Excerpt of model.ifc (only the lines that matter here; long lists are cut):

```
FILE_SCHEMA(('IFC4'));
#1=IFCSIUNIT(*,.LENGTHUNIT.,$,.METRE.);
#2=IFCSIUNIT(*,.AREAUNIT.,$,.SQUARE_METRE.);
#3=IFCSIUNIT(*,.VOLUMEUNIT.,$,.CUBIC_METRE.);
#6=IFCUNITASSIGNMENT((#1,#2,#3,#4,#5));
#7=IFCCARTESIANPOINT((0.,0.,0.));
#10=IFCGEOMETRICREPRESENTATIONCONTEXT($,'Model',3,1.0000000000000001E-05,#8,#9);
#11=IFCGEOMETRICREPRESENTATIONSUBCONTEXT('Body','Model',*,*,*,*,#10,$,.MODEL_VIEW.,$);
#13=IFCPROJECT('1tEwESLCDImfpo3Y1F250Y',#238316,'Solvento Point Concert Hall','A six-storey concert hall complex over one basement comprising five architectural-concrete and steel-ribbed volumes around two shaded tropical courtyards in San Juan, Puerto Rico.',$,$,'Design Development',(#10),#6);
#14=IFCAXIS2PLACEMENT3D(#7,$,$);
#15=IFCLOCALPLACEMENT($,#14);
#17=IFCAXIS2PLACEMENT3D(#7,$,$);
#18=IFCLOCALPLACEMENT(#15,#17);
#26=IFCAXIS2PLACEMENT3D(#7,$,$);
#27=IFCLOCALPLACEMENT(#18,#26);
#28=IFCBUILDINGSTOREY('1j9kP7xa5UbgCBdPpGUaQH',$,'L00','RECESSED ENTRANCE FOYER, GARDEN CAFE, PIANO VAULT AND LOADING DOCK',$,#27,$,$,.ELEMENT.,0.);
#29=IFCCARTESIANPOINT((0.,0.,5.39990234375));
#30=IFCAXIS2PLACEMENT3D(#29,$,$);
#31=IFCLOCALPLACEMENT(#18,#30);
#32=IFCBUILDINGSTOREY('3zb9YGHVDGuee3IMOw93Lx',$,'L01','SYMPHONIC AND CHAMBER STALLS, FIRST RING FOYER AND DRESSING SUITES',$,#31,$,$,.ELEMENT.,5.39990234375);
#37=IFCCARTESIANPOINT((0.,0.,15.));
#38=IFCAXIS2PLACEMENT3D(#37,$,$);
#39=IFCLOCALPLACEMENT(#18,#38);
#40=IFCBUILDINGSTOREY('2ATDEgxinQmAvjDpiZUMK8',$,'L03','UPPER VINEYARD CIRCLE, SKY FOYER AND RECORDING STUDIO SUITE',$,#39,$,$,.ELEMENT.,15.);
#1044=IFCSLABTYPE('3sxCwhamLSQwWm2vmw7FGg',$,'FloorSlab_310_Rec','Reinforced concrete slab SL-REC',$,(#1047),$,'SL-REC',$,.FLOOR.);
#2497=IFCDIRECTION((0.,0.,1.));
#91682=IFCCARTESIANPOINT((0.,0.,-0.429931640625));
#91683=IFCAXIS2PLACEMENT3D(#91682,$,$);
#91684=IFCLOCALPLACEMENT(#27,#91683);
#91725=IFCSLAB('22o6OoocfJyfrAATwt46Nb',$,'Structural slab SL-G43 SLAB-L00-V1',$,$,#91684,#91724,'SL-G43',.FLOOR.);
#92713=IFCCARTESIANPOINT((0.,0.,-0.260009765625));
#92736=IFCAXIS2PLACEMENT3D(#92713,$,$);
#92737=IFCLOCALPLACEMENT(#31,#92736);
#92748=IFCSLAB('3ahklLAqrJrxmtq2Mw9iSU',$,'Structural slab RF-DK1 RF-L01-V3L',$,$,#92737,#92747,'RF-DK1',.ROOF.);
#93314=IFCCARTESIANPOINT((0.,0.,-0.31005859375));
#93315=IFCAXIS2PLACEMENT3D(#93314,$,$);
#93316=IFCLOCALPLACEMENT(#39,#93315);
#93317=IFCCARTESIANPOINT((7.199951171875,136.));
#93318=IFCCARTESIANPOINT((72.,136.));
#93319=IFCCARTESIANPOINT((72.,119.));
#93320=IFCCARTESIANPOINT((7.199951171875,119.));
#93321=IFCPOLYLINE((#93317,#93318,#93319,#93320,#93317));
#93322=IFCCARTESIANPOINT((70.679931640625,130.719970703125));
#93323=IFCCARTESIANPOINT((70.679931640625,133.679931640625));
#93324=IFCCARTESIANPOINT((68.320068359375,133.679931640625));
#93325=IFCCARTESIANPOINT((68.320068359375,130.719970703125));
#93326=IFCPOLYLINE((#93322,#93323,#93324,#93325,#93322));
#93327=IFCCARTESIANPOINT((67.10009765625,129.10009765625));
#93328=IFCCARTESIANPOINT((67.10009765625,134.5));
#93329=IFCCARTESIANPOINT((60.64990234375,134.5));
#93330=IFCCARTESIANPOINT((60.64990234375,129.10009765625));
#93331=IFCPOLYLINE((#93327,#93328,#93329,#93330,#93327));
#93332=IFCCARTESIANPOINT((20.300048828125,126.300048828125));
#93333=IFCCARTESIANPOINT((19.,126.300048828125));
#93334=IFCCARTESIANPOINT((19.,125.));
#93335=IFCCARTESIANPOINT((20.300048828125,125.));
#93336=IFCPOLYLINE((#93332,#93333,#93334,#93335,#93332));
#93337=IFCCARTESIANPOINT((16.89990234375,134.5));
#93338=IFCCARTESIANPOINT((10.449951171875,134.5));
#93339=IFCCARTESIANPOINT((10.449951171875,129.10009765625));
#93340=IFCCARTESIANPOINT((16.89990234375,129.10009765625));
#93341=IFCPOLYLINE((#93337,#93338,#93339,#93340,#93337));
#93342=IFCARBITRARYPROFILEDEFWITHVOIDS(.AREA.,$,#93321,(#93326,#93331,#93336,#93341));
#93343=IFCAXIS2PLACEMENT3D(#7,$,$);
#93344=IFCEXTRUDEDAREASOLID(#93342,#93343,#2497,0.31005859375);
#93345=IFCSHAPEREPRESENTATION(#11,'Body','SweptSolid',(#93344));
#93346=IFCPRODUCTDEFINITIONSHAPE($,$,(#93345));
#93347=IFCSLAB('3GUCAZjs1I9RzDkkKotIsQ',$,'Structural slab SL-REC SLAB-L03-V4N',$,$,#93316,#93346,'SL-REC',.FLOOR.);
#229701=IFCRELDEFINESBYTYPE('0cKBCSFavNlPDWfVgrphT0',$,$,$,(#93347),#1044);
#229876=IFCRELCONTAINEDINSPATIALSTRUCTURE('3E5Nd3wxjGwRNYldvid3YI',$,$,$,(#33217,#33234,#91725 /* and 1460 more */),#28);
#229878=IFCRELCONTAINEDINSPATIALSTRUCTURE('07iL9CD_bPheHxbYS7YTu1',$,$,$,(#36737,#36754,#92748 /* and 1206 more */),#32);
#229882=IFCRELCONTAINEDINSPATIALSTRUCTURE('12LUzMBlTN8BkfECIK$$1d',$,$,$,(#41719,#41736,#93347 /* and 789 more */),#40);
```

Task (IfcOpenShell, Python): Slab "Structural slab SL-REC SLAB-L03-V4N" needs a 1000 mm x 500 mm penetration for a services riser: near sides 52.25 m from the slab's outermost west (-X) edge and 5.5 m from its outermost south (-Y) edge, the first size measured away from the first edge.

```python
import numpy as np
import ifcopenshell
import ifcopenshell.api.feature
import ifcopenshell.api.geometry
import ifcopenshell.api.root
import ifcopenshell.geom
import ifcopenshell.util.placement
import ifcopenshell.util.representation
import ifcopenshell.util.shape
import ifcopenshell.util.unit

model = ifcopenshell.open("model.ifc")
unit_scale = ifcopenshell.util.unit.calculate_unit_scale(model)
settings = ifcopenshell.geom.settings()


def volume(element):
    """Net volume in cubic metres, openings subtracted."""
    shape = ifcopenshell.geom.create_shape(settings, element)
    return ifcopenshell.util.shape.get_volume(shape.geometry)


slab = model.by_id(93347)
before = volume(slab)

# Extent in the slab's own axes, in metres. The edges named are its -X and -Y sides.
slab_shape = ifcopenshell.geom.create_shape(settings, slab)
vertices = ifcopenshell.util.shape.get_vertices(slab_shape.geometry)
x_min, y_min, bottom = vertices.min(axis=0)
top = vertices[:, 2].max()

opening = ifcopenshell.api.root.create_entity(model, ifc_class="IfcOpeningElement", name="Services riser opening", predefined_type="OPENING")
context = ifcopenshell.util.representation.get_context(model, "Model", "Body", "MODEL_VIEW")
width, depth = 1, 0.5
outline = [(0.0, 0.0), (width, 0.0), (width, depth), (0.0, depth), (0.0, 0.0)]
# Overshoot both faces by 50 mm so the cut is clean.
shape = ifcopenshell.api.geometry.add_slab_representation(
    model, context=context, depth=top - bottom + 0.1, polyline=outline
)
ifcopenshell.api.geometry.assign_representation(model, product=opening, representation=shape)

matrix = ifcopenshell.util.placement.get_local_placement(slab.ObjectPlacement)
matrix[:, 3] = matrix @ np.append(np.array([x_min + 52.25, y_min + 5.5, bottom - 0.05]) / unit_scale, 1.0)
ifcopenshell.api.geometry.edit_object_placement(model, product=opening, matrix=matrix, is_si=False)
ifcopenshell.api.feature.add_feature(model, feature=opening, element=slab)

after = volume(slab)

print(f"slab volume {before:.3f} -> {after:.3f} m3")

model.write("model_rev.ifc")
```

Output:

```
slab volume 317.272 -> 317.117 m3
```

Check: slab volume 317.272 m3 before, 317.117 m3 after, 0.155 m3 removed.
